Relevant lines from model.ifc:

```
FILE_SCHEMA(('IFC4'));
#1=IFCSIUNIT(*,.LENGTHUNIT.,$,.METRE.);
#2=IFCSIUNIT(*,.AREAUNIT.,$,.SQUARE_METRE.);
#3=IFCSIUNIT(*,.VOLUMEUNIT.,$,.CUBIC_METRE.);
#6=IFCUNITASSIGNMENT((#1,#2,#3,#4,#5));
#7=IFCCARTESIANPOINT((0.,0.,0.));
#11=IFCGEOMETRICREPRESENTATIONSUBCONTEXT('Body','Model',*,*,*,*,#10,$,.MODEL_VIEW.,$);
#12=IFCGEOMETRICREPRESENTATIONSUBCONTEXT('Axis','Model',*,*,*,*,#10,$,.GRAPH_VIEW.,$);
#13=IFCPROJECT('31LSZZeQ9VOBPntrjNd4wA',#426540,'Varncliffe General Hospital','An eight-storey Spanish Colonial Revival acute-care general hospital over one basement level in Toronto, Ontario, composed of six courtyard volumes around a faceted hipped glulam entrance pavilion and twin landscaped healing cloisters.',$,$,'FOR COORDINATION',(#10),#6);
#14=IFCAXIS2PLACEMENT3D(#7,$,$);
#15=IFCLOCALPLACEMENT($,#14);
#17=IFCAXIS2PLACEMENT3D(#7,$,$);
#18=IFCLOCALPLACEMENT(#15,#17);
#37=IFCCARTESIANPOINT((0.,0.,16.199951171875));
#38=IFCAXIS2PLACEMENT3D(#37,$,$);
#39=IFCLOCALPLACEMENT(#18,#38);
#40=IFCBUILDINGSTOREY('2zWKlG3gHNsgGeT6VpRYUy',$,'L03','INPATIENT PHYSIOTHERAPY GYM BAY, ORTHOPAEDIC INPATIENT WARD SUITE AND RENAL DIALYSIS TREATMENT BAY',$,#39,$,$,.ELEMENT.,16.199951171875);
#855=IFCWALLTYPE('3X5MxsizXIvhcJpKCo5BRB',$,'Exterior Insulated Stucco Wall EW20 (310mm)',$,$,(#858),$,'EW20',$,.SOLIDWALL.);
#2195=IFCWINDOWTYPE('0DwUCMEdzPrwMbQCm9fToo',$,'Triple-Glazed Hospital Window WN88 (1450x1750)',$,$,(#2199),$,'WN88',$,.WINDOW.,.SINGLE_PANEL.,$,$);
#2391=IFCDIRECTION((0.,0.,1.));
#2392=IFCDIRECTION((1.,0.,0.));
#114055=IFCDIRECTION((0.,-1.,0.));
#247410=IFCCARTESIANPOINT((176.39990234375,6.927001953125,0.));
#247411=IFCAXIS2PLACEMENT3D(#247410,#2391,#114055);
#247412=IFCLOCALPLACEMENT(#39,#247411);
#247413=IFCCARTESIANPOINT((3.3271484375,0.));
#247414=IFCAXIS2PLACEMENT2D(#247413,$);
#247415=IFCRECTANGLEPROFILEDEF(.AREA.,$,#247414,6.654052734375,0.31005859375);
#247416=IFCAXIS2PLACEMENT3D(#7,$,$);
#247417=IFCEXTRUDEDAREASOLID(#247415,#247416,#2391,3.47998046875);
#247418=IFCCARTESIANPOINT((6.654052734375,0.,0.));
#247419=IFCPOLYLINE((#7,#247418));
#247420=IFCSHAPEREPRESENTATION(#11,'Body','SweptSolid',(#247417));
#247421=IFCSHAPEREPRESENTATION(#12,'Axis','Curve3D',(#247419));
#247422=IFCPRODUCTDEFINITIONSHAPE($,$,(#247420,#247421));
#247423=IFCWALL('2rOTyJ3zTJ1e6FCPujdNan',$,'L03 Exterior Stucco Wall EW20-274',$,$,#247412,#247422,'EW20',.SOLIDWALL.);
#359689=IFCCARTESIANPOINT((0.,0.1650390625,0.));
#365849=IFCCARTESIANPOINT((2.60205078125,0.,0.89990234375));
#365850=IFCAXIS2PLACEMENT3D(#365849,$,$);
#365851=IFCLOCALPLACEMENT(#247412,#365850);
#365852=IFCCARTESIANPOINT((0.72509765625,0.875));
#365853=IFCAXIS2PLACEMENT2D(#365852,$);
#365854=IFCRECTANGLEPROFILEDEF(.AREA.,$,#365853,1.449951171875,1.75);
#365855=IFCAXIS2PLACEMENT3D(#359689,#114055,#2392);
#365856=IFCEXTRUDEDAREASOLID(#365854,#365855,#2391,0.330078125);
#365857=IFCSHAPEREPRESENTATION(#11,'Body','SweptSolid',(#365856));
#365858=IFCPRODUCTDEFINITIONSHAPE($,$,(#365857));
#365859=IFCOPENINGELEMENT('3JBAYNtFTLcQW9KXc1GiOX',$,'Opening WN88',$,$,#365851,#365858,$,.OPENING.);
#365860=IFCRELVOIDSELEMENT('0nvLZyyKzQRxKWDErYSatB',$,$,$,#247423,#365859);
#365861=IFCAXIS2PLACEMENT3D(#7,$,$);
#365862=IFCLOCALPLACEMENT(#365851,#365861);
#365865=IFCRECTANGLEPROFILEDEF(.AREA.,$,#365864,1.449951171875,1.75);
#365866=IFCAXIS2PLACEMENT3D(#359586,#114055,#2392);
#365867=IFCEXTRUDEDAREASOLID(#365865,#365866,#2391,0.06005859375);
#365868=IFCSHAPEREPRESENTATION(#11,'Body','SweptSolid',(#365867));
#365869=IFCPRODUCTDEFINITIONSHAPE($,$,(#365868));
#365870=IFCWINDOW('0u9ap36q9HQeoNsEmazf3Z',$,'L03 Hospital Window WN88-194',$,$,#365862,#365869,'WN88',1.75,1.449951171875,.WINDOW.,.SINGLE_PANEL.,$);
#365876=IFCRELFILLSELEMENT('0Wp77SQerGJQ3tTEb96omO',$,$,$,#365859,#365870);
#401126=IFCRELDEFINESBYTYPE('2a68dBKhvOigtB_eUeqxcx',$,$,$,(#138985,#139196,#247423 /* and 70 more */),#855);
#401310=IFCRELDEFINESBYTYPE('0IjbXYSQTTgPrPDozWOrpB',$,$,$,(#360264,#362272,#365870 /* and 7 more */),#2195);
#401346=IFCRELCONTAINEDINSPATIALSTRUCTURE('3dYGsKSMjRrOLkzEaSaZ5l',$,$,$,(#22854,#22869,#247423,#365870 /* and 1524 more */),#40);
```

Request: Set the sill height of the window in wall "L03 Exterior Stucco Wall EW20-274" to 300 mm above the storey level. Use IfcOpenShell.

```python
import numpy as np
import ifcopenshell
import ifcopenshell.api.geometry
import ifcopenshell.geom
import ifcopenshell.util.element
import ifcopenshell.util.placement
import ifcopenshell.util.shape
import ifcopenshell.util.unit

model = ifcopenshell.open("model.ifc")
unit_scale = ifcopenshell.util.unit.calculate_unit_scale(model)

window = model.by_guid("0u9ap36q9HQeoNsEmazf3Z")
opening = window.FillsVoids[0].RelatingOpeningElement
storey = ifcopenshell.util.element.get_container(window, ifc_class="IfcBuildingStorey")
level = ifcopenshell.util.placement.get_local_placement(storey.ObjectPlacement)[2, 3]

# The opening's origin need not be at the sill, so measure its lowest point.
shape = ifcopenshell.geom.create_shape(ifcopenshell.geom.settings(), opening)
bottom = ifcopenshell.util.shape.get_shape_bottom_elevation(shape, shape.geometry) / unit_scale
dz = level + 0.3 / unit_scale - bottom

shift = np.array([0.0, 0.0, dz])
# The window is placed relative to its opening, so it follows when the opening moves.
matrix = ifcopenshell.util.placement.get_local_placement(opening.ObjectPlacement)
matrix[:3, 3] += shift
ifcopenshell.api.geometry.edit_object_placement(
    model, product=opening, matrix=matrix, is_si=False, should_transform_children=True
)

print(f"moved by {dz * unit_scale:+.3f} m")

model.write("model_updated.ifc")
```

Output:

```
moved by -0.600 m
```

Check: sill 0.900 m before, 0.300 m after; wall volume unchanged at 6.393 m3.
